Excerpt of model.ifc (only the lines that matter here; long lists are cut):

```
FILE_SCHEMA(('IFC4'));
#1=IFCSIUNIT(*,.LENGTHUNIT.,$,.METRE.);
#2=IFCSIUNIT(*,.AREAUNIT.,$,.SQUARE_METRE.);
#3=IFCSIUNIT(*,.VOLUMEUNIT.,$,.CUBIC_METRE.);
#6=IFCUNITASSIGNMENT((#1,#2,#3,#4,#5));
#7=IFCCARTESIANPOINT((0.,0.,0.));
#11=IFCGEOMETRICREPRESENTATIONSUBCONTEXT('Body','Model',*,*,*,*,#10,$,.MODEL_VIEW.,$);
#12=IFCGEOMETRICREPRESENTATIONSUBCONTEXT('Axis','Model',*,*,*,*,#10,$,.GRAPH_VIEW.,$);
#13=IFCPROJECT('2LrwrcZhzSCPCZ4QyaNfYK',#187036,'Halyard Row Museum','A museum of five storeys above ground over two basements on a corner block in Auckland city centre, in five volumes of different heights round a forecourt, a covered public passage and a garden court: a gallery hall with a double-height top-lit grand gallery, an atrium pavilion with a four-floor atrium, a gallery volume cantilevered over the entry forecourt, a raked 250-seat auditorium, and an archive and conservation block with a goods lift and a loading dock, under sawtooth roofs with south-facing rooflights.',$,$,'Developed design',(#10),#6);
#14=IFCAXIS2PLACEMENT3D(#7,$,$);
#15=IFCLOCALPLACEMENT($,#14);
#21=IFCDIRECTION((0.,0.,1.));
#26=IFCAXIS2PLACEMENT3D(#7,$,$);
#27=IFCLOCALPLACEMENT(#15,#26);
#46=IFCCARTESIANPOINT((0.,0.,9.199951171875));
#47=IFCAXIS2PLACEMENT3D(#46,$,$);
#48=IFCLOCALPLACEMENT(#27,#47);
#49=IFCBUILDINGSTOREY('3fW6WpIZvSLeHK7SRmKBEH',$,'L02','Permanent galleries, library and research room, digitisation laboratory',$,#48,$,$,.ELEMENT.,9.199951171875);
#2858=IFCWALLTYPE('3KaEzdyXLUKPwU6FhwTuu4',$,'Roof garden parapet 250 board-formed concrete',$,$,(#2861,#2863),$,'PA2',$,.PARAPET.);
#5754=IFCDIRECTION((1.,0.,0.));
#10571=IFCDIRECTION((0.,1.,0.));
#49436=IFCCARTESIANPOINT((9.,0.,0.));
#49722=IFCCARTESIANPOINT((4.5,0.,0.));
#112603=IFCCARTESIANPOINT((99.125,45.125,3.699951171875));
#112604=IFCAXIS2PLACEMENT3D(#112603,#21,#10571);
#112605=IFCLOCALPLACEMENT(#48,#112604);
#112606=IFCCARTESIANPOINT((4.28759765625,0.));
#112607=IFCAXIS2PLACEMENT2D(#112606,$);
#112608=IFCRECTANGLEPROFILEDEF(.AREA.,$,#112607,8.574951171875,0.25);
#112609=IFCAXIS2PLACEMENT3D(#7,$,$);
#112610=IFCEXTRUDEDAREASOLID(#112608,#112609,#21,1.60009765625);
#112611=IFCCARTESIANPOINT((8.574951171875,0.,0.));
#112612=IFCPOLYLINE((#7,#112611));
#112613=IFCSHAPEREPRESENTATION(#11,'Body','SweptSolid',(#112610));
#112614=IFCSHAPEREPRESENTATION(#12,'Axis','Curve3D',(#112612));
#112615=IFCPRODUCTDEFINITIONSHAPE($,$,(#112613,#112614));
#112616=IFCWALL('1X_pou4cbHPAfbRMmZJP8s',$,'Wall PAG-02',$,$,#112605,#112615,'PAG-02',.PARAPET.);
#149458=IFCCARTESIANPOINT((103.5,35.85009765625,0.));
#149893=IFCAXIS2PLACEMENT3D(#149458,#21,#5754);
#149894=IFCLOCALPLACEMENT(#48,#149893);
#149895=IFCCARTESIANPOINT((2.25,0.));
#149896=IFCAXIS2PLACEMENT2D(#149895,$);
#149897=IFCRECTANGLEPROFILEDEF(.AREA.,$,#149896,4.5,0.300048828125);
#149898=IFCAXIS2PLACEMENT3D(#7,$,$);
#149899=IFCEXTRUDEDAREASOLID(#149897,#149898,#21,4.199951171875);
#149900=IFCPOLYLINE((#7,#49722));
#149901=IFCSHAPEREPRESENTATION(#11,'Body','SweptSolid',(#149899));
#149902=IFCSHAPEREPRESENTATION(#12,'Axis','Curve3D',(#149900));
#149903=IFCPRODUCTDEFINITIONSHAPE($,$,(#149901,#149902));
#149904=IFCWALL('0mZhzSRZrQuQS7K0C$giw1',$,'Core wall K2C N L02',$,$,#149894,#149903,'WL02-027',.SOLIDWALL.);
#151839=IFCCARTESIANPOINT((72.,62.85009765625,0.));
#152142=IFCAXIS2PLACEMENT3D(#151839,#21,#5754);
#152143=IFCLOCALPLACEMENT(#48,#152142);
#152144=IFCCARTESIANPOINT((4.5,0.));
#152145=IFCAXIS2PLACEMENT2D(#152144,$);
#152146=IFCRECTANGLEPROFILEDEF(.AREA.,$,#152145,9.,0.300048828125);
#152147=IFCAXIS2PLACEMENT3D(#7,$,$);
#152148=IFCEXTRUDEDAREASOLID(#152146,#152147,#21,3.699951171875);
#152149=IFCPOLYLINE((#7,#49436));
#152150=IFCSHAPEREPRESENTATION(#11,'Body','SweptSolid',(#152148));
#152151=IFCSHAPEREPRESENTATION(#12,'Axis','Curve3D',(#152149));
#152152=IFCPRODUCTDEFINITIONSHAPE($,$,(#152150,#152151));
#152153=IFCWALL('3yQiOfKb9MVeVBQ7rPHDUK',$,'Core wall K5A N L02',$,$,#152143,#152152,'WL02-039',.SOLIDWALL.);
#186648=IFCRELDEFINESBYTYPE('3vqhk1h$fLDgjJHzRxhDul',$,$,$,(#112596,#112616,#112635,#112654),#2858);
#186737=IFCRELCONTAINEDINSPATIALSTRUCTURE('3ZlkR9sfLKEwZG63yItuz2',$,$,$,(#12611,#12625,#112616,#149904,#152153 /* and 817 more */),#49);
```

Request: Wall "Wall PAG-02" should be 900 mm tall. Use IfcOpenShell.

```python
import ifcopenshell
import ifcopenshell.geom
import ifcopenshell.util.representation
import ifcopenshell.util.shape
import ifcopenshell.util.unit

model = ifcopenshell.open("model.ifc")
unit_scale = ifcopenshell.util.unit.calculate_unit_scale(model)
settings = ifcopenshell.geom.settings()


def volume(element):
    """Net volume in cubic metres, openings subtracted."""
    shape = ifcopenshell.geom.create_shape(settings, element)
    return ifcopenshell.util.shape.get_volume(shape.geometry)


wall = model.by_guid("1X_pou4cbHPAfbRMmZJP8s")
before = volume(wall)

body = ifcopenshell.util.representation.get_representation(wall, "Model", "Body")
solid = body.Items[0]
old_height = solid.Depth
solid.Depth = 0.9 / unit_scale
after = volume(wall)

print(f"height {old_height:g} -> {solid.Depth:g}, volume {before:.3f} -> {after:.3f} m3")

model.write("model-out.ifc")
```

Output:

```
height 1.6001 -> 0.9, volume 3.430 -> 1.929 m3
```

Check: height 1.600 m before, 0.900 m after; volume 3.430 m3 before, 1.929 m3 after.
